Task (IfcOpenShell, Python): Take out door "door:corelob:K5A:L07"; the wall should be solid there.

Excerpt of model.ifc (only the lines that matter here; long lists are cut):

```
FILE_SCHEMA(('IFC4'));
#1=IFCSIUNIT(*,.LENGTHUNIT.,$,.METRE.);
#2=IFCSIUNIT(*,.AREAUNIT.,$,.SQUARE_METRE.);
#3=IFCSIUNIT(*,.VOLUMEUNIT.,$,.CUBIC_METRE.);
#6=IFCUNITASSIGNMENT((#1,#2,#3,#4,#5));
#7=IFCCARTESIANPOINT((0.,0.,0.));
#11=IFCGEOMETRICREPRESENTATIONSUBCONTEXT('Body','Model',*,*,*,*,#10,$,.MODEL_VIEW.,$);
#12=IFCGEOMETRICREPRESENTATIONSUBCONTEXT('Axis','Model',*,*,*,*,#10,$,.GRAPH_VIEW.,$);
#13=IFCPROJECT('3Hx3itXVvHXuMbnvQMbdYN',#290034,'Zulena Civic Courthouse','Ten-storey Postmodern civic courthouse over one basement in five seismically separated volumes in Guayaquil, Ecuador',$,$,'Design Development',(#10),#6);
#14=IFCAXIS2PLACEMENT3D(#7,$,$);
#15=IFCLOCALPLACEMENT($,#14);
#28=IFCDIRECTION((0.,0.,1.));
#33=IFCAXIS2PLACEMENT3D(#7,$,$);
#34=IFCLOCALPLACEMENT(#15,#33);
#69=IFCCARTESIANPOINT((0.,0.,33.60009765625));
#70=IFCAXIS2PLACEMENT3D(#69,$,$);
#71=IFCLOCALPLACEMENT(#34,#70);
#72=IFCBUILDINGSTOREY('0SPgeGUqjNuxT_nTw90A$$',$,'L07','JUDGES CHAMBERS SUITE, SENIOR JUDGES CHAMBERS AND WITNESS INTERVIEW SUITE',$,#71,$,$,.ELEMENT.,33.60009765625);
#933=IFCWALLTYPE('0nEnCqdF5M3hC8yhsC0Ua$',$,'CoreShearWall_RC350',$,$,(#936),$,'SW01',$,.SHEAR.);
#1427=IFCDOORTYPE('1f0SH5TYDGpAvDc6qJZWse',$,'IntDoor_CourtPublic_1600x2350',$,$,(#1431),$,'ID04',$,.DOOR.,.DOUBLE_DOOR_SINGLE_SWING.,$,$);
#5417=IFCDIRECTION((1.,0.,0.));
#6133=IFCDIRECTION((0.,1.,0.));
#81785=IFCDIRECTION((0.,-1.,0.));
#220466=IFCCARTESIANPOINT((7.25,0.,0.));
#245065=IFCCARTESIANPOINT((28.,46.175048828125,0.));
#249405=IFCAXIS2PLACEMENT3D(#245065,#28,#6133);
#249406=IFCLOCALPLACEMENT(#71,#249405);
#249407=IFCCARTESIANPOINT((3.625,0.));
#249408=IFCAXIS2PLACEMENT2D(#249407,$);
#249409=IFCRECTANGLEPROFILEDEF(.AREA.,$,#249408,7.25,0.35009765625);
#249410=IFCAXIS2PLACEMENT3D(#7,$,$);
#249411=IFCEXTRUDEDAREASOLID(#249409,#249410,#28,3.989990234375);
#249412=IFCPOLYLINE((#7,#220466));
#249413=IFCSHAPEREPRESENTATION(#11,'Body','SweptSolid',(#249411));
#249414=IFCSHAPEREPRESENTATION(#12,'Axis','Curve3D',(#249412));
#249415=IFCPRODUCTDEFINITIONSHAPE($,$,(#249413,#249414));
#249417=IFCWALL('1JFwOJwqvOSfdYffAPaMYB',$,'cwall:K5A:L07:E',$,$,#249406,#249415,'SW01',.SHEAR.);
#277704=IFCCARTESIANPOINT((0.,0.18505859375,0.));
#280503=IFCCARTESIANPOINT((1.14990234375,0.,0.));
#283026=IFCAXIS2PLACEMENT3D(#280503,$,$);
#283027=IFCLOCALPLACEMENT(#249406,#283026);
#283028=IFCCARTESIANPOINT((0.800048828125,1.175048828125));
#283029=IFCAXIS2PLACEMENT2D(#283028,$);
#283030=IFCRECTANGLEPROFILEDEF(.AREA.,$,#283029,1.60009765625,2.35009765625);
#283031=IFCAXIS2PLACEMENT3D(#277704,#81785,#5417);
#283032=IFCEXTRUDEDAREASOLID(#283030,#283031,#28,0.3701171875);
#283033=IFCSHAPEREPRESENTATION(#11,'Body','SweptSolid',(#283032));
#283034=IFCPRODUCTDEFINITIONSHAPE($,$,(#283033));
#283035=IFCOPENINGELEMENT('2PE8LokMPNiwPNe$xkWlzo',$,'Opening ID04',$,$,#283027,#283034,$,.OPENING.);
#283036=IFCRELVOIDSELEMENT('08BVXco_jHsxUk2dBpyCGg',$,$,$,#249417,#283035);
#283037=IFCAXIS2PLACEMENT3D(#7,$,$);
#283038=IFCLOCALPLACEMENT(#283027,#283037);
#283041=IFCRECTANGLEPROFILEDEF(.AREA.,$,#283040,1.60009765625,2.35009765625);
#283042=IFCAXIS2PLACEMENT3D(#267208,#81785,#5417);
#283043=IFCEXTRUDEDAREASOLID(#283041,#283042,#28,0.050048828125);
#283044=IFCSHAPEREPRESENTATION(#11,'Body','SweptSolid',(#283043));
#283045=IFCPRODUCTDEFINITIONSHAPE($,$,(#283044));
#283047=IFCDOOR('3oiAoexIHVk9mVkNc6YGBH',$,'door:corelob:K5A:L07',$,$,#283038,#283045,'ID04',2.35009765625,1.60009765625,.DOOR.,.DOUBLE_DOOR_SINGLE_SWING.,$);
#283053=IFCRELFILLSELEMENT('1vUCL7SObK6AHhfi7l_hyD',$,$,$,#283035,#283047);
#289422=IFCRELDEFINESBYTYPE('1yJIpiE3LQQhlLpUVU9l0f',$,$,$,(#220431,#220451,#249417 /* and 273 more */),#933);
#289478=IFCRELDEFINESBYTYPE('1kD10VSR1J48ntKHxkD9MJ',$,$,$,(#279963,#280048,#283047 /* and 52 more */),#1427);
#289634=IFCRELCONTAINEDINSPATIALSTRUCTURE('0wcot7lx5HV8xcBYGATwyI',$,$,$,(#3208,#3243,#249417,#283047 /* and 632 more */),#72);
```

```python
import ifcopenshell
import ifcopenshell.api.feature
import ifcopenshell.api.root
import ifcopenshell.geom
import ifcopenshell.util.shape

model = ifcopenshell.open("model.ifc")
settings = ifcopenshell.geom.settings()


def volume(element):
    """Net volume in cubic metres, openings subtracted."""
    shape = ifcopenshell.geom.create_shape(settings, element)
    return ifcopenshell.util.shape.get_volume(shape.geometry)


door = model.by_guid("3oiAoexIHVk9mVkNc6YGBH")
opening = door.FillsVoids[0].RelatingOpeningElement
wall = opening.VoidsElements[0].RelatingBuildingElement
before = volume(wall)

ifcopenshell.api.root.remove_product(model, product=door)
ifcopenshell.api.feature.remove_feature(model, feature=opening)

after = volume(wall)

print(f"wall volume {before:.3f} -> {after:.3f} m3")

model.write("model_v2.ifc")
```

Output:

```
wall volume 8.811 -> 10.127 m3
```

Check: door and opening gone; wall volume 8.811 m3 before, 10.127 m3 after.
